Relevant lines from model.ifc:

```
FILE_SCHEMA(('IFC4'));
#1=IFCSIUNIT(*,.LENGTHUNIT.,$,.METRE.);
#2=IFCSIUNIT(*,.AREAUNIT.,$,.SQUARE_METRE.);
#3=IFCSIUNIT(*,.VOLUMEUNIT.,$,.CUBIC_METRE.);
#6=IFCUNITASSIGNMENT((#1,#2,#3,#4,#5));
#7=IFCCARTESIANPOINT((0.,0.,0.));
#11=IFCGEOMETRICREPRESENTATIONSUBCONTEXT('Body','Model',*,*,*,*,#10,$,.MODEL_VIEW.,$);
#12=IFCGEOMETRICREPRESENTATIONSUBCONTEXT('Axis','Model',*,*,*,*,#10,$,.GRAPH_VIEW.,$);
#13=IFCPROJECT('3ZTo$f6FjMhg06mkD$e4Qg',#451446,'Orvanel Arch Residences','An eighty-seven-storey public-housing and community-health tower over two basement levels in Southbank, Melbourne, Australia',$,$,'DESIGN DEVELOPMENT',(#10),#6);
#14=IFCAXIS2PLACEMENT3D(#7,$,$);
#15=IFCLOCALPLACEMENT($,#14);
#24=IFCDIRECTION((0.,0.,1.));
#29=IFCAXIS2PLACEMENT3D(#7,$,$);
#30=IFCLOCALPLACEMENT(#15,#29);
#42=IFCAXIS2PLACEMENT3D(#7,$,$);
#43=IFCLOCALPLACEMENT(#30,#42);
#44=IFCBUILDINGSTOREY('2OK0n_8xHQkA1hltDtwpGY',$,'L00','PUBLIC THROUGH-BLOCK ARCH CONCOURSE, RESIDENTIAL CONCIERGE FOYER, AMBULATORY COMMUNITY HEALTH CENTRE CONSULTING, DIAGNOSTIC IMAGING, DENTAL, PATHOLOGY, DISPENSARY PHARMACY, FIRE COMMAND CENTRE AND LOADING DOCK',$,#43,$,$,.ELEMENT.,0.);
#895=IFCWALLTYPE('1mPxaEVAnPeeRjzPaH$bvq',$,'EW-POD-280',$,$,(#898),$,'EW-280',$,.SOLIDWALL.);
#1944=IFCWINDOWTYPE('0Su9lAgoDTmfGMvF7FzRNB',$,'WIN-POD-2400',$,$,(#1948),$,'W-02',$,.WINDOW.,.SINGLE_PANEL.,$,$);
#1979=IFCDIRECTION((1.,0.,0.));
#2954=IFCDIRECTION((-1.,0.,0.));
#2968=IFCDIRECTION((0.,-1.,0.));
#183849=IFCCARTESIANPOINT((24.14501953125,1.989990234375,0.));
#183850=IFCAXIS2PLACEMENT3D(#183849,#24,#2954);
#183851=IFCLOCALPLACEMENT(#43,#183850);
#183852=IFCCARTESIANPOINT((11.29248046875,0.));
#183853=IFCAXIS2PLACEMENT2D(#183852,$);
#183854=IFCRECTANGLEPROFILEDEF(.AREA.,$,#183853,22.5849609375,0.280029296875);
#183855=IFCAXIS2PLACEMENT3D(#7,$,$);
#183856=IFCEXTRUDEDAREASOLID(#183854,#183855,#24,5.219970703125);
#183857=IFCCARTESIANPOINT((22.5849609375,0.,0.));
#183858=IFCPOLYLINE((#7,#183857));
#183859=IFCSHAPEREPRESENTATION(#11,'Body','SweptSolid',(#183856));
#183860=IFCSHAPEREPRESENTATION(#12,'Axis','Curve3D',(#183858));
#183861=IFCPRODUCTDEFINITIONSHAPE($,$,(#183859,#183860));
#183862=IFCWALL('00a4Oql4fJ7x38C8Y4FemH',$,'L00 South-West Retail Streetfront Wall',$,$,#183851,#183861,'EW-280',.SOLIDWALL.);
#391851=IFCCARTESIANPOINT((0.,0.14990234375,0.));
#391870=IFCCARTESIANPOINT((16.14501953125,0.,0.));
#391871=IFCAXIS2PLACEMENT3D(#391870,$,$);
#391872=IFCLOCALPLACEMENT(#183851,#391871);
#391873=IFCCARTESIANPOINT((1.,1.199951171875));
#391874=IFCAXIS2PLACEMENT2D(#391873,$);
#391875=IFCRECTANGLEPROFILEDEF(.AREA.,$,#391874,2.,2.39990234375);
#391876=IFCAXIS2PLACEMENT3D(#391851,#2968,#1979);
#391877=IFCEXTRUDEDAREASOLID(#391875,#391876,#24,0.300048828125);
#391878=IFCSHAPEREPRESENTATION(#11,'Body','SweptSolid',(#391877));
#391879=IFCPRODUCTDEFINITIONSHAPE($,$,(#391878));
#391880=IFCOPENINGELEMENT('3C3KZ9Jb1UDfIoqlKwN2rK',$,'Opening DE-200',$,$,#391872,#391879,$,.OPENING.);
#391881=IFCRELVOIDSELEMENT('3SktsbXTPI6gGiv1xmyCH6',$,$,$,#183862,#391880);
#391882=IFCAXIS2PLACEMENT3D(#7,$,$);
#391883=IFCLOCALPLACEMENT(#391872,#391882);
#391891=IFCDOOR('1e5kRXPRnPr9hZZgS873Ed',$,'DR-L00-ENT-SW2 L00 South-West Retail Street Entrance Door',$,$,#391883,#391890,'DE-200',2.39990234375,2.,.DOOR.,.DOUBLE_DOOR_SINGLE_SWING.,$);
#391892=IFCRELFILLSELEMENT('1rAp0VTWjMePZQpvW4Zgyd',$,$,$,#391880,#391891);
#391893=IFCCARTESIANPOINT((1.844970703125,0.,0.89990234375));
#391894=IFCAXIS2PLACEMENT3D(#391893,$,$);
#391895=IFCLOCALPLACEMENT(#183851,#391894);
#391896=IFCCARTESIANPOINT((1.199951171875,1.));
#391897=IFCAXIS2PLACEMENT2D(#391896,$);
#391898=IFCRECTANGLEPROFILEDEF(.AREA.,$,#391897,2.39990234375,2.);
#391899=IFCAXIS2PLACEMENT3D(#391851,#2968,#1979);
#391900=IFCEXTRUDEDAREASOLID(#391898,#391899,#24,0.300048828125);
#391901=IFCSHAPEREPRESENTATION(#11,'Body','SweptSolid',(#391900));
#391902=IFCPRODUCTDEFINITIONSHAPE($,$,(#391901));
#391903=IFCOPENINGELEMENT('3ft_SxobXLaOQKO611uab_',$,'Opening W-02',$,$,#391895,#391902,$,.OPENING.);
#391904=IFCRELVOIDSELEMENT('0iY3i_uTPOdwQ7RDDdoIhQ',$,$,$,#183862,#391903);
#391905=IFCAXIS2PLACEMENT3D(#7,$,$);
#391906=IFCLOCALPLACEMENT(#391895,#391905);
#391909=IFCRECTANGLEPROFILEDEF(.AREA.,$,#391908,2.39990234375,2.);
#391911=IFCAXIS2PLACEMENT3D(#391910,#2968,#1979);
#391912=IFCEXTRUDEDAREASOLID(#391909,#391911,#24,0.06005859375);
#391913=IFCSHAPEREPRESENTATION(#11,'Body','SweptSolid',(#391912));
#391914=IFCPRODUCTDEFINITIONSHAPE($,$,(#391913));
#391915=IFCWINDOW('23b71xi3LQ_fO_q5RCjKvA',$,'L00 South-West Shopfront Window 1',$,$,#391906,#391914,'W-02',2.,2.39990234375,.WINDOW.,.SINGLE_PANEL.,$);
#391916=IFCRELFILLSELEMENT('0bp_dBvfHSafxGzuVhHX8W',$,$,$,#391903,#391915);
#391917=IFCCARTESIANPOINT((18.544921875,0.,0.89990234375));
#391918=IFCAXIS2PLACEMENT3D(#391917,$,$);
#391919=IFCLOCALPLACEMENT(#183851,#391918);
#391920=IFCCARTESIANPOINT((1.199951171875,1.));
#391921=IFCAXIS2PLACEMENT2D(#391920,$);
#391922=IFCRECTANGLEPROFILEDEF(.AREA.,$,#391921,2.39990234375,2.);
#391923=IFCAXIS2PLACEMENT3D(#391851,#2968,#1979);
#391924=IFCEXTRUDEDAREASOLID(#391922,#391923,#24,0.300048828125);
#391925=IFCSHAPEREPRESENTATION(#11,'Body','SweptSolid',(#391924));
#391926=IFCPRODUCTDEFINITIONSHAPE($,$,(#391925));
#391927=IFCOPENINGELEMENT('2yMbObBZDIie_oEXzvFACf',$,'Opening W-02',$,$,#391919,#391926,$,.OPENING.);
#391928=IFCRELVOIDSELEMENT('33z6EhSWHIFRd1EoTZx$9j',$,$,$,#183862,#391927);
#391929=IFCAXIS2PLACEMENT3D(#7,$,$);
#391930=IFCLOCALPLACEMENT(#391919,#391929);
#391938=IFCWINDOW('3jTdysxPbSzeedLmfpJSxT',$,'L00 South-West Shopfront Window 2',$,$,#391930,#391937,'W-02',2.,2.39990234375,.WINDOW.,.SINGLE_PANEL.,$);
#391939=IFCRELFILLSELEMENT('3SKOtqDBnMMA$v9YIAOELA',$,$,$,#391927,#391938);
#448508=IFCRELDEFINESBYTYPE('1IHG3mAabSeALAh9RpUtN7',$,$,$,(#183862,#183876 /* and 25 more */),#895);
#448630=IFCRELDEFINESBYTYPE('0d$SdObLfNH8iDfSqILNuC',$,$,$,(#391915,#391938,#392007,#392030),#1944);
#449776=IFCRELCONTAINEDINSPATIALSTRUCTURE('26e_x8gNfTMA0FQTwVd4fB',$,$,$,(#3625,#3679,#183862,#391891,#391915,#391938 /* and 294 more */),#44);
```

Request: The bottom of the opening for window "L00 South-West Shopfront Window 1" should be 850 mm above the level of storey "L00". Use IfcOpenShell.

```python
import numpy as np
import ifcopenshell
import ifcopenshell.api.geometry
import ifcopenshell.geom
import ifcopenshell.util.element
import ifcopenshell.util.placement
import ifcopenshell.util.shape
import ifcopenshell.util.unit

model = ifcopenshell.open("model.ifc")
unit_scale = ifcopenshell.util.unit.calculate_unit_scale(model)

window = model.by_id(391915)
opening = window.FillsVoids[0].RelatingOpeningElement
storey = ifcopenshell.util.element.get_container(window, ifc_class="IfcBuildingStorey")
level = ifcopenshell.util.placement.get_local_placement(storey.ObjectPlacement)[2, 3]

# The opening's origin need not be at the sill, so measure its lowest point.
shape = ifcopenshell.geom.create_shape(ifcopenshell.geom.settings(), opening)
bottom = ifcopenshell.util.shape.get_shape_bottom_elevation(shape, shape.geometry) / unit_scale
dz = level + 0.85 / unit_scale - bottom

shift = np.array([0.0, 0.0, dz])
# The window is placed relative to its opening, so it follows when the opening moves.
matrix = ifcopenshell.util.placement.get_local_placement(opening.ObjectPlacement)
matrix[:3, 3] += shift
ifcopenshell.api.geometry.edit_object_placement(
    model, product=opening, matrix=matrix, is_si=False, should_transform_children=True
)

print(f"moved by {dz * unit_scale:+.3f} m")

model.write("model_updated.ifc")
```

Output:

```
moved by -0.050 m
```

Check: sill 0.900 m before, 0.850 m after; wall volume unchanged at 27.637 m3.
